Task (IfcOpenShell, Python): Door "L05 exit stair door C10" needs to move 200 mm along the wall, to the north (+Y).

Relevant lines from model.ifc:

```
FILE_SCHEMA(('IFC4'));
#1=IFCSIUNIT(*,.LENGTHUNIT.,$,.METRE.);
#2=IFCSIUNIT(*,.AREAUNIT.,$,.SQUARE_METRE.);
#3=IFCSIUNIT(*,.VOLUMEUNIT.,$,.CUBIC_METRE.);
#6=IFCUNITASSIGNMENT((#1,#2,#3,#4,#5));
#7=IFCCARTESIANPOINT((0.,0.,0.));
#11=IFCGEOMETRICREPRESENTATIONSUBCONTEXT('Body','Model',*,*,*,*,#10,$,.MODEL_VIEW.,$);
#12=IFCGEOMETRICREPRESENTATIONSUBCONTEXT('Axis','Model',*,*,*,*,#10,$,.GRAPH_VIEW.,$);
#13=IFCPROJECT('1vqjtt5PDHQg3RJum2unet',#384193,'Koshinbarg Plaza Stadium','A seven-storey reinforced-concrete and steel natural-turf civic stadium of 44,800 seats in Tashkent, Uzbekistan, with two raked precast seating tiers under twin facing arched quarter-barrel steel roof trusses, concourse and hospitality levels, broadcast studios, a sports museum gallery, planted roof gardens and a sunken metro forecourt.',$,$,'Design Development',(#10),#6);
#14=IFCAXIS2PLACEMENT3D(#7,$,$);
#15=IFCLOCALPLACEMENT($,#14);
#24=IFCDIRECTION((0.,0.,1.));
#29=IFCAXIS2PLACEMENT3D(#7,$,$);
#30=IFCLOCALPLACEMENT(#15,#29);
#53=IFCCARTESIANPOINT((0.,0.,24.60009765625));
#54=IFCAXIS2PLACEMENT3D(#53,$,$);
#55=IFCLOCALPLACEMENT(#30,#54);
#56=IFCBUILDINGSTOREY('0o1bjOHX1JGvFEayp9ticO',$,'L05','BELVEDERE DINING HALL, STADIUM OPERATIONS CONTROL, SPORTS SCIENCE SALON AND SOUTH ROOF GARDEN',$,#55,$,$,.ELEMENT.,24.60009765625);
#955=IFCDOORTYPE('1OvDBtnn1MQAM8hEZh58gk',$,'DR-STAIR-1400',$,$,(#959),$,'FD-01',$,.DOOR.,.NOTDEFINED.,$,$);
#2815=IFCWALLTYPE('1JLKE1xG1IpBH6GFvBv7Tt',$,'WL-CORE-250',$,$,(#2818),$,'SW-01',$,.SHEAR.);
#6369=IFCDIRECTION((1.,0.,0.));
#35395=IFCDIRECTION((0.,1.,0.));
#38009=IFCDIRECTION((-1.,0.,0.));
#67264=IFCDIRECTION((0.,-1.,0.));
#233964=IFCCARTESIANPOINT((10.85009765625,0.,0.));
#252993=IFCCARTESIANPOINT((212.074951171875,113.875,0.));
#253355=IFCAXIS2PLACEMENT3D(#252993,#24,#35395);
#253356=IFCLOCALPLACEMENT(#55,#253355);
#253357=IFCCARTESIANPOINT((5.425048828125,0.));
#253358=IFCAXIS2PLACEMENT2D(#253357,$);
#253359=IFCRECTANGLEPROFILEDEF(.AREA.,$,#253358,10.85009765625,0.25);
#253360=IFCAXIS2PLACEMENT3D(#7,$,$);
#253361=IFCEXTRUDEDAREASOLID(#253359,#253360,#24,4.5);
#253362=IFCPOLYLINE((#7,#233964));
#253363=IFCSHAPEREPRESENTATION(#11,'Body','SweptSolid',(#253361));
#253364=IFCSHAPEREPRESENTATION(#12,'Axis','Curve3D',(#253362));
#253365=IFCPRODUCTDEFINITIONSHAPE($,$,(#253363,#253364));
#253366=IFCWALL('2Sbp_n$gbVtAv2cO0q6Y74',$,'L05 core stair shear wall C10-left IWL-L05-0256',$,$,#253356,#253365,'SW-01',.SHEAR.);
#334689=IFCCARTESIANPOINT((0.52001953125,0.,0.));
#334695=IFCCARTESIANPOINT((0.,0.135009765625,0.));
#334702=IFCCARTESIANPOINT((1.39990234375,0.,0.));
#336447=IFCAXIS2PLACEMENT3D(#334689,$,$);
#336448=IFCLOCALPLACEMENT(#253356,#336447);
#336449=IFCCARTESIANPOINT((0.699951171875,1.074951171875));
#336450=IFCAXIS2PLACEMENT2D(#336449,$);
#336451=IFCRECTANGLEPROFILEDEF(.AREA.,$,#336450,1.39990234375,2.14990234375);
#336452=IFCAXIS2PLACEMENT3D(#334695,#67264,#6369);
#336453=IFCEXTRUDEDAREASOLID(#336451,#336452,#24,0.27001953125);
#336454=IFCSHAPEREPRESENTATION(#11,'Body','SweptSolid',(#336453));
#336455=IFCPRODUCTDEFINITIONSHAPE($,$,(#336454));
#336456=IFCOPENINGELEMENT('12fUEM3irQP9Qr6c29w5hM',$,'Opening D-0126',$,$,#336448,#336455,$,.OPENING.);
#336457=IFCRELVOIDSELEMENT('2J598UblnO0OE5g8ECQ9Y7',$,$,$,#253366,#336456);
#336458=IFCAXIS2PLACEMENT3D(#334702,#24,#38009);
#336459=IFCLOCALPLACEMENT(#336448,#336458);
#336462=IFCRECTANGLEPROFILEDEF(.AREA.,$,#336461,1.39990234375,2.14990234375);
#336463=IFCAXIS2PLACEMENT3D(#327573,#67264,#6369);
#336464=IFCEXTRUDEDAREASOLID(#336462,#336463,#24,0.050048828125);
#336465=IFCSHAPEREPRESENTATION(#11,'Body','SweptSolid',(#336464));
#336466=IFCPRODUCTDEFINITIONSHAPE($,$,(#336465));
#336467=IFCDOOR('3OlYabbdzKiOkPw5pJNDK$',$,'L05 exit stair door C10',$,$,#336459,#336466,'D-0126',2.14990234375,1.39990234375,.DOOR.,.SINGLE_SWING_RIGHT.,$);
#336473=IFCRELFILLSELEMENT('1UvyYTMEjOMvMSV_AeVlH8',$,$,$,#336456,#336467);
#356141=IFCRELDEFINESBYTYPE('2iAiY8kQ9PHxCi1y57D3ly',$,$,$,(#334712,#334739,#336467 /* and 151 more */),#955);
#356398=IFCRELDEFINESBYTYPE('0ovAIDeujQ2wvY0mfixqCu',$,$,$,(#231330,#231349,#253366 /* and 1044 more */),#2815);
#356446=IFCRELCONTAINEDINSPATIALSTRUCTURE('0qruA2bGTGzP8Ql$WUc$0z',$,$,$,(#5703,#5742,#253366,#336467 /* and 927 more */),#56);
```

```python
import ifcopenshell
import ifcopenshell.api.geometry
import ifcopenshell.util.placement
import ifcopenshell.util.unit

model = ifcopenshell.open("model.ifc")
unit_scale = ifcopenshell.util.unit.calculate_unit_scale(model)

door = model.by_id(336467)
opening = door.FillsVoids[0].RelatingOpeningElement
wall = opening.VoidsElements[0].RelatingBuildingElement

wall_matrix = ifcopenshell.util.placement.get_local_placement(wall.ObjectPlacement)
shift = wall_matrix[:3, 0] * 0.2 / unit_scale
before = ifcopenshell.util.placement.get_local_placement(door.ObjectPlacement)[:3, 3].copy()

# The door is placed relative to its opening, so it follows when the opening moves.
matrix = ifcopenshell.util.placement.get_local_placement(opening.ObjectPlacement)
matrix[:3, 3] += shift
ifcopenshell.api.geometry.edit_object_placement(
    model, product=opening, matrix=matrix, is_si=False, should_transform_children=True
)

after = ifcopenshell.util.placement.get_local_placement(door.ObjectPlacement)[:3, 3]
print("door moved by", (after - before).round(3) + 0.0)

model.write("model_edited.ifc")
```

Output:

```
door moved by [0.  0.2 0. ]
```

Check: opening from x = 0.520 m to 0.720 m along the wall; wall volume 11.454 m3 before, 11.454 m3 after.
